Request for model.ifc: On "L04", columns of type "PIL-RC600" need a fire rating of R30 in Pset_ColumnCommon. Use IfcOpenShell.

First a look at what the model holds.

```python
import ifcopenshell
import ifcopenshell.util.element

model = ifcopenshell.open("model.ifc")
print(model.schema)
storey = next(s for s in model.by_type("IfcBuildingStorey") if s.Name == "L04")
columns = [e for e in ifcopenshell.util.element.get_decomposition(storey) if e.is_a("IfcColumn")]
seen = {}
for e in columns:
    element_type = ifcopenshell.util.element.get_type(e)
    key = (element_type.Name if element_type != e and element_type else None, ifcopenshell.util.element.get_pset(e, "Pset_ColumnCommon", "FireRating"))
    seen[key] = seen.get(key, 0) + 1
for (name, value), count in sorted(seen.items(), key=str):
    print(count, "x", name, "|", value)
```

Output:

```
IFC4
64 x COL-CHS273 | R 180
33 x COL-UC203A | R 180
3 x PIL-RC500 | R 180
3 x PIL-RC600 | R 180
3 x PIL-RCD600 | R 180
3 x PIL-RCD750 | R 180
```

```python
import ifcopenshell
import ifcopenshell.api.pset
import ifcopenshell.util.element

model = ifcopenshell.open("model.ifc")

storey = next(s for s in model.by_type("IfcBuildingStorey") if s.Name == "L04")
columns = [e for e in ifcopenshell.util.element.get_decomposition(storey) if e.is_a("IfcColumn")]

count = 0
for e in columns:
    element_type = ifcopenshell.util.element.get_type(e)
    if element_type in (None, e) or element_type.Name != "PIL-RC600":
        continue
    # add_pset returns the element's existing set when there is one.
    pset = ifcopenshell.api.pset.add_pset(model, product=e, name="Pset_ColumnCommon")
    ifcopenshell.api.pset.edit_pset(model, pset=pset, properties={"FireRating": "R30"})
    count += 1

print(count, "columns updated")

model.write("model_edited.ifc")
```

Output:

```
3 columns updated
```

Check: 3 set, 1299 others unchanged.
